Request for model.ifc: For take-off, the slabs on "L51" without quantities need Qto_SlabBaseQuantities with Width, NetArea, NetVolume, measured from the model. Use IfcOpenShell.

First a look at what the model holds.

```python
import ifcopenshell
import ifcopenshell.util.element
import ifcopenshell.util.unit

model = ifcopenshell.open("model.ifc")
print(model.schema)
for unit_type in ("LENGTHUNIT", "AREAUNIT", "VOLUMEUNIT"):
    print(unit_type, ifcopenshell.util.unit.calculate_unit_scale(model, unit_type))
storey = next(s for s in model.by_type("IfcBuildingStorey") if s.Name == "L51")
slabs = [e for e in ifcopenshell.util.element.get_decomposition(storey) if e.is_a("IfcSlab")]
for e in sorted(slabs, key=lambda e: e.id()):
    print(e.id(), e.is_a(), e.Name, list(ifcopenshell.util.element.get_psets(e, qtos_only=True)), sep=" | ")
```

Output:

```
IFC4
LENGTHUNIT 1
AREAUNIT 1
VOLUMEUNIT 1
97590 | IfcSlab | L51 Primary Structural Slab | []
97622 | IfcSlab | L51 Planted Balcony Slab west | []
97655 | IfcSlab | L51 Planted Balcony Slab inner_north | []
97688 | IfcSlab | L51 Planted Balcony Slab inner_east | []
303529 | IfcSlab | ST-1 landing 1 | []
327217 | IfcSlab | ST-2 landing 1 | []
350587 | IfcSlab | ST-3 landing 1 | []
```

```python
import ifcopenshell
import ifcopenshell.api.pset
import ifcopenshell.geom
import ifcopenshell.util.element
import ifcopenshell.util.shape
import ifcopenshell.util.unit

model = ifcopenshell.open("model.ifc")
unit_scale = ifcopenshell.util.unit.calculate_unit_scale(model)
area_scale = ifcopenshell.util.unit.calculate_unit_scale(model, "AREAUNIT")
volume_scale = ifcopenshell.util.unit.calculate_unit_scale(model, "VOLUMEUNIT")
settings = ifcopenshell.geom.settings()

storey = next(s for s in model.by_type("IfcBuildingStorey") if s.Name == "L51")
slabs = [e for e in ifcopenshell.util.element.get_decomposition(storey) if e.is_a("IfcSlab")]

for e in sorted(slabs, key=lambda e: e.id()):
    if ifcopenshell.util.element.get_psets(e, qtos_only=True, should_inherit=False):
        continue
    # Geometry comes back in metres, in the element's own axes.
    shape = ifcopenshell.geom.create_shape(settings, e)
    values = {
        "Width": ifcopenshell.util.shape.get_z(shape.geometry) / unit_scale,
        "NetArea": ifcopenshell.util.shape.get_footprint_area(shape.geometry) / area_scale,
        "NetVolume": ifcopenshell.util.shape.get_volume(shape.geometry) / volume_scale,
    }
    qto = ifcopenshell.api.pset.add_qto(model, product=e, name="Qto_SlabBaseQuantities")
    ifcopenshell.api.pset.edit_qto(model, qto=qto, properties=values)
    print(e.id(), {k: round(v, 3) for k, v in values.items()})

model.write("model_rev.ifc")
```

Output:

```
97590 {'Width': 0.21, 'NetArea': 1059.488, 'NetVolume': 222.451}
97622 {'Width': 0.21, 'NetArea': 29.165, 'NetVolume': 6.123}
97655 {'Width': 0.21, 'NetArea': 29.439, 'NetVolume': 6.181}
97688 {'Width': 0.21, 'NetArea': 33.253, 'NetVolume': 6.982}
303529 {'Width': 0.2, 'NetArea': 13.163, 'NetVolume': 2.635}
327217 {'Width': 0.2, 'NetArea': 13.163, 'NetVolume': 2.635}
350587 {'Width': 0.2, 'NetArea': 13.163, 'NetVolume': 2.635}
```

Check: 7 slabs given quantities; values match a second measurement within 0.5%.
